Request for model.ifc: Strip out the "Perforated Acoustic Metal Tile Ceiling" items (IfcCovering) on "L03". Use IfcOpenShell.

First a look at what the model holds.

```python
import ifcopenshell
import ifcopenshell.util.element

model = ifcopenshell.open("model.ifc")
print(model.schema)
storey = next(s for s in model.by_type("IfcBuildingStorey") if s.Name == "L03")
coverings = [e for e in ifcopenshell.util.element.get_decomposition(storey) if e.is_a("IfcCovering")]
seen = {}
for e in coverings:
    element_type = ifcopenshell.util.element.get_type(e)
    name = element_type.Name if element_type not in (None, e) else None
    seen[name] = seen.get(name, 0) + 1
for name, count in sorted(seen.items(), key=str):
    print(count, "x", name)
```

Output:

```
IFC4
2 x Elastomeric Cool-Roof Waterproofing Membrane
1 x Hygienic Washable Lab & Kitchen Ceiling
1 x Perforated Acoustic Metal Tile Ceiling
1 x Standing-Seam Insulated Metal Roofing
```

```python
import ifcopenshell
import ifcopenshell.api.root
import ifcopenshell.util.element

model = ifcopenshell.open("model.ifc")

storey = next(s for s in model.by_type("IfcBuildingStorey") if s.Name == "L03")
coverings = [e for e in ifcopenshell.util.element.get_decomposition(storey) if e.is_a("IfcCovering")]
targets = [e for e in coverings if (t := ifcopenshell.util.element.get_type(e)) not in (None, e) and t.Name == "Perforated Acoustic Metal Tile Ceiling"]

for e in targets:
    ifcopenshell.api.root.remove_product(model, product=e)
print(len(targets), "removed")

model.write("model_updated.ifc")
```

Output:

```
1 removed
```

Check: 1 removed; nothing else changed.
